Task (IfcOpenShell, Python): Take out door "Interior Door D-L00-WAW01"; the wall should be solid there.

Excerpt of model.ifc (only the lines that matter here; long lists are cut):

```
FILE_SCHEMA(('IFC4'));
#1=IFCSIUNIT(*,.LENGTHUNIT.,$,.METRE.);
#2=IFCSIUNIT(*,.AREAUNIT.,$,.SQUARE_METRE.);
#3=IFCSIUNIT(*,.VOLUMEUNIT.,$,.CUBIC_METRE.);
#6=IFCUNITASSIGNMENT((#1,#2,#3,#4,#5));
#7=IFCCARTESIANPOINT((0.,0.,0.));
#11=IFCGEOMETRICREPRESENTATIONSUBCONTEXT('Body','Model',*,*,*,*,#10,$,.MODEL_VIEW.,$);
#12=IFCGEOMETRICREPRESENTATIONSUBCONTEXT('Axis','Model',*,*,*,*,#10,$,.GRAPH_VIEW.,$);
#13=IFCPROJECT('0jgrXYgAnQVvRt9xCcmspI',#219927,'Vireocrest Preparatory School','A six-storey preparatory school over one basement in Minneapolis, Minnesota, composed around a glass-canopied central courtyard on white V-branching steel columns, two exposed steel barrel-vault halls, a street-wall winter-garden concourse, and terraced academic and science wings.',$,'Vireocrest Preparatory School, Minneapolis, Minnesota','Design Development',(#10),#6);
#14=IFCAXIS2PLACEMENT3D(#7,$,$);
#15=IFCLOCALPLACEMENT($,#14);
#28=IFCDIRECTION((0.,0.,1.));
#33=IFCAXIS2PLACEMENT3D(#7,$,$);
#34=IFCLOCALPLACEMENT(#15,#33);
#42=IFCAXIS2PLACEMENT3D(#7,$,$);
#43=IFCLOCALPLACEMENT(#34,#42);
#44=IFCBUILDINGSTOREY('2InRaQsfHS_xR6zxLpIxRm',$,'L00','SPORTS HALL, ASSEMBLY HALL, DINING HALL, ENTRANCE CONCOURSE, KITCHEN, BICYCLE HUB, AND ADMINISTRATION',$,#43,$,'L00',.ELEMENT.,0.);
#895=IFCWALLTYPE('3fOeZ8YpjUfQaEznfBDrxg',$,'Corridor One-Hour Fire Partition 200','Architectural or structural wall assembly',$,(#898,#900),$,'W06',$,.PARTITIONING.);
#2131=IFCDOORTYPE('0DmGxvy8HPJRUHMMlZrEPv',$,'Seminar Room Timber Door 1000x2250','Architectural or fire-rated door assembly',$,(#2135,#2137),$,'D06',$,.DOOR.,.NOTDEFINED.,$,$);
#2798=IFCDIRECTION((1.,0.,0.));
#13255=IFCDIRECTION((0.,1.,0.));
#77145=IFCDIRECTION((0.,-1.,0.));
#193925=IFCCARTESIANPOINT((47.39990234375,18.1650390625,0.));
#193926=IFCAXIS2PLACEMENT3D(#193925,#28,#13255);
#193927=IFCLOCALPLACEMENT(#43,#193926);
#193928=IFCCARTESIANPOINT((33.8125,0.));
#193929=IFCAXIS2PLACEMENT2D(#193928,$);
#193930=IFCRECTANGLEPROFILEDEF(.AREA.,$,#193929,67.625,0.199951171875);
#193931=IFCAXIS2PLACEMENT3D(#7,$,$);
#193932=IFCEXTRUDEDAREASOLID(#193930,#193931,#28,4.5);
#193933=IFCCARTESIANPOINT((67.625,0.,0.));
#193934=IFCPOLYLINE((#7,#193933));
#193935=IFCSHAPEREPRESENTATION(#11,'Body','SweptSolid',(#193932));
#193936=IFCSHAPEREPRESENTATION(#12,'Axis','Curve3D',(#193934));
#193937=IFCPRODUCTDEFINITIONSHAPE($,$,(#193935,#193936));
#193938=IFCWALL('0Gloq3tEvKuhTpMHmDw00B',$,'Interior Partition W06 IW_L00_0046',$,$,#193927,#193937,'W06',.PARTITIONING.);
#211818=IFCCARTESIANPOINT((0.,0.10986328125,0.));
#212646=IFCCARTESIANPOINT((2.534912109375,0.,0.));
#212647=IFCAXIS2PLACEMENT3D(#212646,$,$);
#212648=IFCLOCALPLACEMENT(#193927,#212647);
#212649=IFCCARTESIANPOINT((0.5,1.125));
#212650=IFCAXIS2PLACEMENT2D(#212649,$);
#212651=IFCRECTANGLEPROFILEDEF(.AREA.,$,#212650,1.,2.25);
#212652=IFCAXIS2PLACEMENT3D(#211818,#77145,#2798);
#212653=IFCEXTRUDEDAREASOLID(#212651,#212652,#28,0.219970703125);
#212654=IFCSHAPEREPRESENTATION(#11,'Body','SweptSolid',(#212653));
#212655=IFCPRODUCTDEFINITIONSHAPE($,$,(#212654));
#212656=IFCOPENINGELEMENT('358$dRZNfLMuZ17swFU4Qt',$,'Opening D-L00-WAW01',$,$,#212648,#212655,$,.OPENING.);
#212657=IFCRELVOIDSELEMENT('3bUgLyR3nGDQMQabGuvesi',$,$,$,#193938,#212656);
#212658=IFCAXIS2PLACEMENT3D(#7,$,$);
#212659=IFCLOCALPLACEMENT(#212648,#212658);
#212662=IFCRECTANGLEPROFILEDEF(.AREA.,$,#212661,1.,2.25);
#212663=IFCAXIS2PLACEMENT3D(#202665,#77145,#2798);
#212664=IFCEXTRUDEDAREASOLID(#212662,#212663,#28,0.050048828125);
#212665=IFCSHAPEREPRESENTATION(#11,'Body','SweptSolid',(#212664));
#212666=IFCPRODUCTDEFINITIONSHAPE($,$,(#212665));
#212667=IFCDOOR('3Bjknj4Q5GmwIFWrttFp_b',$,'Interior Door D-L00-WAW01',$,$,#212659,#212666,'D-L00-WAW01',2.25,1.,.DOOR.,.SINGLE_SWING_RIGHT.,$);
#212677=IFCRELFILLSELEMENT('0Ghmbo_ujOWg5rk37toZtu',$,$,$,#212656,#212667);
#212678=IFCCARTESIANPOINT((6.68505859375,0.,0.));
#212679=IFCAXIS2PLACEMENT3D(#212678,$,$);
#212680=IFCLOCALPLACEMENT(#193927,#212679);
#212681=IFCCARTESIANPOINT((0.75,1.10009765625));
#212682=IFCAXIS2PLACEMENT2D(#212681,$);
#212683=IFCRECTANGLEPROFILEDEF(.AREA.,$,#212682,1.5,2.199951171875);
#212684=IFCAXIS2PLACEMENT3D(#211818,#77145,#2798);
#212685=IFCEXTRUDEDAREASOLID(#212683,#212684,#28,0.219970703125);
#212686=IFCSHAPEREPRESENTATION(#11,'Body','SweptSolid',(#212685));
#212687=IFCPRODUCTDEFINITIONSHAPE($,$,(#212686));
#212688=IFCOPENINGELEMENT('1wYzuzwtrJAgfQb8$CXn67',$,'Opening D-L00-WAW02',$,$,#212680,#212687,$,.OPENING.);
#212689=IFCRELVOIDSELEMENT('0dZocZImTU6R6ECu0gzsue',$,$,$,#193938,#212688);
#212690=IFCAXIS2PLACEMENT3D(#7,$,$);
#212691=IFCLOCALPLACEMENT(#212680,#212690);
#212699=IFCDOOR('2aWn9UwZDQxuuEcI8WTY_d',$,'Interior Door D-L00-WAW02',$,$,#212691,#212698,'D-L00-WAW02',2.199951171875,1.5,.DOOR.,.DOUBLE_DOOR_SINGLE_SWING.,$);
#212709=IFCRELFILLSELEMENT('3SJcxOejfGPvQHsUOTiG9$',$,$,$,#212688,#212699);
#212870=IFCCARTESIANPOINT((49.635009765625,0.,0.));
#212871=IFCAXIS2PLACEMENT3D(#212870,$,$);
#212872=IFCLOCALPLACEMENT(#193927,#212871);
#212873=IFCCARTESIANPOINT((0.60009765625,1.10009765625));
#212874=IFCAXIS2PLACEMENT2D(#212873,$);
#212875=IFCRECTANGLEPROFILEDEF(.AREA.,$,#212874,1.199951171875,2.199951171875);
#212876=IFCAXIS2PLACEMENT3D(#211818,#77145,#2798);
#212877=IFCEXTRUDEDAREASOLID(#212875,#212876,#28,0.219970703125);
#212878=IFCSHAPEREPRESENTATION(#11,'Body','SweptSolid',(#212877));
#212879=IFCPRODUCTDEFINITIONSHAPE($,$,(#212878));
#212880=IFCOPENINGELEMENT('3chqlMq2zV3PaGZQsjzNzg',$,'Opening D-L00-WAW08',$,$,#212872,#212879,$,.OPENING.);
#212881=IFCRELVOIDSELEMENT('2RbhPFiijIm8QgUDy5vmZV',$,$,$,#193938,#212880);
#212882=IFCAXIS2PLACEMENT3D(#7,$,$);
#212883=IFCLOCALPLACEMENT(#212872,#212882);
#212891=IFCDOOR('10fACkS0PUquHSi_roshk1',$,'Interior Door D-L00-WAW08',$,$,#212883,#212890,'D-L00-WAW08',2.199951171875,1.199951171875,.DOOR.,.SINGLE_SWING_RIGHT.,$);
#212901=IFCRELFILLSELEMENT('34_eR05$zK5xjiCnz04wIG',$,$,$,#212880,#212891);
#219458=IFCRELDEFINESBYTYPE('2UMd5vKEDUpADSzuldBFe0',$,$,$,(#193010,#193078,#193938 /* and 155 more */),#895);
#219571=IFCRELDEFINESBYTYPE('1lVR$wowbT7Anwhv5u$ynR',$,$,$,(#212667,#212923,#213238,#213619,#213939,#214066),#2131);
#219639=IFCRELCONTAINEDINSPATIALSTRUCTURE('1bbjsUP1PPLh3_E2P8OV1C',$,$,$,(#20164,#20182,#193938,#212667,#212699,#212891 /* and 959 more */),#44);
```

```python
import ifcopenshell
import ifcopenshell.api.feature
import ifcopenshell.api.root
import ifcopenshell.geom
import ifcopenshell.util.shape

model = ifcopenshell.open("model.ifc")
settings = ifcopenshell.geom.settings()


def volume(element):
    """Net volume in cubic metres, openings subtracted."""
    shape = ifcopenshell.geom.create_shape(settings, element)
    return ifcopenshell.util.shape.get_volume(shape.geometry)


door = model.by_guid("3Bjknj4Q5GmwIFWrttFp_b")
opening = door.FillsVoids[0].RelatingOpeningElement
wall = opening.VoidsElements[0].RelatingBuildingElement
before = volume(wall)

ifcopenshell.api.root.remove_product(model, product=door)
ifcopenshell.api.feature.remove_feature(model, feature=opening)

after = volume(wall)

print(f"wall volume {before:.3f} -> {after:.3f} m3")

model.write("model_updated.ifc")
```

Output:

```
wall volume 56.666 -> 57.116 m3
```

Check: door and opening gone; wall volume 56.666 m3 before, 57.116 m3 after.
